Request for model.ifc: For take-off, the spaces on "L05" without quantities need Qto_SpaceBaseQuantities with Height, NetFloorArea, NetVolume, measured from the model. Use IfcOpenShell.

First a look at what the model holds.

```python
import ifcopenshell
import ifcopenshell.util.element
import ifcopenshell.util.unit

model = ifcopenshell.open("model.ifc")
print(model.schema)
for unit_type in ("LENGTHUNIT", "AREAUNIT", "VOLUMEUNIT"):
    print(unit_type, ifcopenshell.util.unit.calculate_unit_scale(model, unit_type))
storey = next(s for s in model.by_type("IfcBuildingStorey") if s.Name == "L05")
spaces = [e for e in ifcopenshell.util.element.get_decomposition(storey) if e.is_a("IfcSpace")]
for e in sorted(spaces, key=lambda e: e.id()):
    print(e.id(), e.is_a(), e.Name, list(ifcopenshell.util.element.get_psets(e, qtos_only=True)), sep=" | ")
```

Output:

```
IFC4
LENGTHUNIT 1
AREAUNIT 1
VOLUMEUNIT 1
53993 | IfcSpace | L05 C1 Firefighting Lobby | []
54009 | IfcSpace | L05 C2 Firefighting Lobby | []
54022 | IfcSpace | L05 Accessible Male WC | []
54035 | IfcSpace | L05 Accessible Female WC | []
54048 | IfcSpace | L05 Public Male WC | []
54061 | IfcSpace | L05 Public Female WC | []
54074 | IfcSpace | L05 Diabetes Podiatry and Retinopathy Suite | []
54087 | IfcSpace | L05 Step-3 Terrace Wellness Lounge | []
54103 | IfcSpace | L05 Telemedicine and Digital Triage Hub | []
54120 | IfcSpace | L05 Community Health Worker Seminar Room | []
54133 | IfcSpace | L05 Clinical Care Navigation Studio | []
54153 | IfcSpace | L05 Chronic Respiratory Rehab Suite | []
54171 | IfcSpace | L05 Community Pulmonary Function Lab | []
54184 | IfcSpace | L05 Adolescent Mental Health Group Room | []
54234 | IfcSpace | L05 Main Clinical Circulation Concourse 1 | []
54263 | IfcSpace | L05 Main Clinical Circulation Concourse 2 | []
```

```python
import ifcopenshell
import ifcopenshell.api.pset
import ifcopenshell.geom
import ifcopenshell.util.element
import ifcopenshell.util.shape
import ifcopenshell.util.unit

model = ifcopenshell.open("model.ifc")
unit_scale = ifcopenshell.util.unit.calculate_unit_scale(model)
area_scale = ifcopenshell.util.unit.calculate_unit_scale(model, "AREAUNIT")
volume_scale = ifcopenshell.util.unit.calculate_unit_scale(model, "VOLUMEUNIT")
settings = ifcopenshell.geom.settings()

storey = next(s for s in model.by_type("IfcBuildingStorey") if s.Name == "L05")
spaces = [e for e in ifcopenshell.util.element.get_decomposition(storey) if e.is_a("IfcSpace")]

for e in sorted(spaces, key=lambda e: e.id()):
    if ifcopenshell.util.element.get_psets(e, qtos_only=True, should_inherit=False):
        continue
    # Geometry comes back in metres, in the element's own axes.
    shape = ifcopenshell.geom.create_shape(settings, e)
    values = {
        "Height": ifcopenshell.util.shape.get_z(shape.geometry) / unit_scale,
        "NetFloorArea": ifcopenshell.util.shape.get_footprint_area(shape.geometry) / area_scale,
        "NetVolume": ifcopenshell.util.shape.get_volume(shape.geometry) / volume_scale,
    }
    qto = ifcopenshell.api.pset.add_qto(model, product=e, name="Qto_SpaceBaseQuantities")
    ifcopenshell.api.pset.edit_qto(model, qto=qto, properties=values)
    print(e.id(), {k: round(v, 3) for k, v in values.items()})

model.write("model-out.ifc")
```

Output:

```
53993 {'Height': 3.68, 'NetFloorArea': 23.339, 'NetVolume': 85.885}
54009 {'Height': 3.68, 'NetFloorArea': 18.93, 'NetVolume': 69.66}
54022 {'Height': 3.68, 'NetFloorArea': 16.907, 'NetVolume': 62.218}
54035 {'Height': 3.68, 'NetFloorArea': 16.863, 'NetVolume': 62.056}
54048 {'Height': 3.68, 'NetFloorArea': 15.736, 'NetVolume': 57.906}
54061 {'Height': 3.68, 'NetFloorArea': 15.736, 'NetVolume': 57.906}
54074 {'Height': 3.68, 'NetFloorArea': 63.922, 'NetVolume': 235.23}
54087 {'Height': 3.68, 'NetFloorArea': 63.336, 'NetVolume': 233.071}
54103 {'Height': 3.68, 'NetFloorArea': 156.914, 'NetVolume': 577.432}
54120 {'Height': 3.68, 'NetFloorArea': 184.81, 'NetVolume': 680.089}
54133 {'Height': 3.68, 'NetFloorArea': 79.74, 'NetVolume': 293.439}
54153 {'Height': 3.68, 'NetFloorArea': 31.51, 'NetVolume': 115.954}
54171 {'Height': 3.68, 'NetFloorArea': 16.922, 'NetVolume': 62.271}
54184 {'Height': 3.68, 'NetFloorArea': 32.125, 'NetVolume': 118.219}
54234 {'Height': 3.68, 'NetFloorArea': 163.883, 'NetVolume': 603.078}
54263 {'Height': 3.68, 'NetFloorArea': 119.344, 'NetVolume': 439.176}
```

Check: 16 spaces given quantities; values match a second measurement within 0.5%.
